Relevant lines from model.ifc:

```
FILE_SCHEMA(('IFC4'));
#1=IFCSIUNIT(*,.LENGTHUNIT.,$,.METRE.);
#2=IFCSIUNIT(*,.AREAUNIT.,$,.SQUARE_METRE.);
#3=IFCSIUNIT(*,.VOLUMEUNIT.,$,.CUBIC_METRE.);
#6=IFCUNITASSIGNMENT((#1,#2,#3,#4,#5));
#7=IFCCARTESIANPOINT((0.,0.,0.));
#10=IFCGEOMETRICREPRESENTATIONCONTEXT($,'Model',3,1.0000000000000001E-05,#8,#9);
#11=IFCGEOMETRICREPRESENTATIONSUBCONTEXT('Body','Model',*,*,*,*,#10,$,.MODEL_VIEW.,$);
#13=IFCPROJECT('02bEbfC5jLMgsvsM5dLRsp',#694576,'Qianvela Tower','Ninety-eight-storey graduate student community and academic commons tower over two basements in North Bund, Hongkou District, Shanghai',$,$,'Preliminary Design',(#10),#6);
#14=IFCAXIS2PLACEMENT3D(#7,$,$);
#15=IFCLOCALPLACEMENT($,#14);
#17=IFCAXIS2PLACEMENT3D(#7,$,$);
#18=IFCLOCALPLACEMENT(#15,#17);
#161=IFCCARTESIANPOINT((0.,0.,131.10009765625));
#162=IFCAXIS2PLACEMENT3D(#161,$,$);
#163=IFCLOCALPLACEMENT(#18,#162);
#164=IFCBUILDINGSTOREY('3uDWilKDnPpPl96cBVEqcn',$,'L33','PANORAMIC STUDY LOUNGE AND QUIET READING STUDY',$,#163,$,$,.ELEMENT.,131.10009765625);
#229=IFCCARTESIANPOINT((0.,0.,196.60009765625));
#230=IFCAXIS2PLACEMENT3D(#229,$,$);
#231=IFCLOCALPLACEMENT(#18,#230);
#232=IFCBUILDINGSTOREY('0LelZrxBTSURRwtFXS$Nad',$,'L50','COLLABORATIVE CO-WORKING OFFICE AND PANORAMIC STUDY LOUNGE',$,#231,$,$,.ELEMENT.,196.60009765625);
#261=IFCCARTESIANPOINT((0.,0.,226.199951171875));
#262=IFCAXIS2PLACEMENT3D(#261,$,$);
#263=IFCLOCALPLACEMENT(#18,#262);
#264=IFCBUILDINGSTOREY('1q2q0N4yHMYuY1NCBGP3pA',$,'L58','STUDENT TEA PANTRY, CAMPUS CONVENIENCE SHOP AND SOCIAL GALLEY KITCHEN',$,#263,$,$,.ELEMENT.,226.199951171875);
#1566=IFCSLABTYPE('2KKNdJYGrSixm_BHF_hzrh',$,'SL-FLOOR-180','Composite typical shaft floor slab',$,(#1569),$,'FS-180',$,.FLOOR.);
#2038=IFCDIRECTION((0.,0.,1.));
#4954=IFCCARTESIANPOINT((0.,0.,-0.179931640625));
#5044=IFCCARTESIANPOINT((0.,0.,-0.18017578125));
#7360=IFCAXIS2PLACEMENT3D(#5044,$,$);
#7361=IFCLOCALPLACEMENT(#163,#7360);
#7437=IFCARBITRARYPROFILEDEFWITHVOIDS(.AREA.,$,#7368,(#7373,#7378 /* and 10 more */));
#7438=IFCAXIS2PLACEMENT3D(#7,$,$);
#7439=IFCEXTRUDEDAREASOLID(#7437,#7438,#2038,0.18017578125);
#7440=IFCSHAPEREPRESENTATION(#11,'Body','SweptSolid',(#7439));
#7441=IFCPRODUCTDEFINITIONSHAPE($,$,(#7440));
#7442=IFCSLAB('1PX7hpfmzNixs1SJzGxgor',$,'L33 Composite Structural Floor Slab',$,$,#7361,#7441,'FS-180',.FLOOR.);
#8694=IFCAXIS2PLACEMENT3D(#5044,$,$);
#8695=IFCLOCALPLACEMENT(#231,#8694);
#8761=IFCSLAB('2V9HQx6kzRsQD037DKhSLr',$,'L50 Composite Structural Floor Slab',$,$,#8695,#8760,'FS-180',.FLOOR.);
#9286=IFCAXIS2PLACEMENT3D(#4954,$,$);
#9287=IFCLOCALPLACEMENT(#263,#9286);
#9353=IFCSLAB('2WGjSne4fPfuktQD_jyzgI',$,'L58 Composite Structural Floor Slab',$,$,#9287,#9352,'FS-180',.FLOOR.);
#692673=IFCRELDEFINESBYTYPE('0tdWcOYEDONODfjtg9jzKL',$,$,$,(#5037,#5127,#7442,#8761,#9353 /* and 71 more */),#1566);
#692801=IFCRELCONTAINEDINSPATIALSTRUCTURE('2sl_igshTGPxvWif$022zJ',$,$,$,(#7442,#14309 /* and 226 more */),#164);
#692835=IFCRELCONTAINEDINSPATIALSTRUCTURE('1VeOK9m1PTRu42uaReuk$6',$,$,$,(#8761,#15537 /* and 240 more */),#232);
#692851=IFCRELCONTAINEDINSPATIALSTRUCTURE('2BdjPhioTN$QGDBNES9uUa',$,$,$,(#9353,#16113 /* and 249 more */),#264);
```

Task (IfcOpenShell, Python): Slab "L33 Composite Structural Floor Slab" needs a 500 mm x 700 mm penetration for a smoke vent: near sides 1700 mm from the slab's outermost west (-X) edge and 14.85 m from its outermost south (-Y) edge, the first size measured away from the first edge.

```python
import numpy as np
import ifcopenshell
import ifcopenshell.api.feature
import ifcopenshell.api.geometry
import ifcopenshell.api.root
import ifcopenshell.geom
import ifcopenshell.util.placement
import ifcopenshell.util.representation
import ifcopenshell.util.shape
import ifcopenshell.util.unit

model = ifcopenshell.open("model.ifc")
unit_scale = ifcopenshell.util.unit.calculate_unit_scale(model)
settings = ifcopenshell.geom.settings()


def volume(element):
    """Net volume in cubic metres, openings subtracted."""
    shape = ifcopenshell.geom.create_shape(settings, element)
    return ifcopenshell.util.shape.get_volume(shape.geometry)


slab = model.by_guid("1PX7hpfmzNixs1SJzGxgor")
before = volume(slab)

# Extent in the slab's own axes, in metres. The edges named are its -X and -Y sides.
slab_shape = ifcopenshell.geom.create_shape(settings, slab)
vertices = ifcopenshell.util.shape.get_vertices(slab_shape.geometry)
x_min, y_min, bottom = vertices.min(axis=0)
top = vertices[:, 2].max()

opening = ifcopenshell.api.root.create_entity(model, ifc_class="IfcOpeningElement", name="Smoke vent opening", predefined_type="OPENING")
context = ifcopenshell.util.representation.get_context(model, "Model", "Body", "MODEL_VIEW")
width, depth = 0.5, 0.7
outline = [(0.0, 0.0), (width, 0.0), (width, depth), (0.0, depth), (0.0, 0.0)]
# Overshoot both faces by 50 mm so the cut is clean.
shape = ifcopenshell.api.geometry.add_slab_representation(
    model, context=context, depth=top - bottom + 0.1, polyline=outline
)
ifcopenshell.api.geometry.assign_representation(model, product=opening, representation=shape)

matrix = ifcopenshell.util.placement.get_local_placement(slab.ObjectPlacement)
matrix[:, 3] = matrix @ np.append(np.array([x_min + 1.7, y_min + 14.85, bottom - 0.05]) / unit_scale, 1.0)
ifcopenshell.api.geometry.edit_object_placement(model, product=opening, matrix=matrix, is_si=False)
ifcopenshell.api.feature.add_feature(model, feature=opening, element=slab)

after = volume(slab)

print(f"slab volume {before:.3f} -> {after:.3f} m3")

model.write("model_v2.ifc")
```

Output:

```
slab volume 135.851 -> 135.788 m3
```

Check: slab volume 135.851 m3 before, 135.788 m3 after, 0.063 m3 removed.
